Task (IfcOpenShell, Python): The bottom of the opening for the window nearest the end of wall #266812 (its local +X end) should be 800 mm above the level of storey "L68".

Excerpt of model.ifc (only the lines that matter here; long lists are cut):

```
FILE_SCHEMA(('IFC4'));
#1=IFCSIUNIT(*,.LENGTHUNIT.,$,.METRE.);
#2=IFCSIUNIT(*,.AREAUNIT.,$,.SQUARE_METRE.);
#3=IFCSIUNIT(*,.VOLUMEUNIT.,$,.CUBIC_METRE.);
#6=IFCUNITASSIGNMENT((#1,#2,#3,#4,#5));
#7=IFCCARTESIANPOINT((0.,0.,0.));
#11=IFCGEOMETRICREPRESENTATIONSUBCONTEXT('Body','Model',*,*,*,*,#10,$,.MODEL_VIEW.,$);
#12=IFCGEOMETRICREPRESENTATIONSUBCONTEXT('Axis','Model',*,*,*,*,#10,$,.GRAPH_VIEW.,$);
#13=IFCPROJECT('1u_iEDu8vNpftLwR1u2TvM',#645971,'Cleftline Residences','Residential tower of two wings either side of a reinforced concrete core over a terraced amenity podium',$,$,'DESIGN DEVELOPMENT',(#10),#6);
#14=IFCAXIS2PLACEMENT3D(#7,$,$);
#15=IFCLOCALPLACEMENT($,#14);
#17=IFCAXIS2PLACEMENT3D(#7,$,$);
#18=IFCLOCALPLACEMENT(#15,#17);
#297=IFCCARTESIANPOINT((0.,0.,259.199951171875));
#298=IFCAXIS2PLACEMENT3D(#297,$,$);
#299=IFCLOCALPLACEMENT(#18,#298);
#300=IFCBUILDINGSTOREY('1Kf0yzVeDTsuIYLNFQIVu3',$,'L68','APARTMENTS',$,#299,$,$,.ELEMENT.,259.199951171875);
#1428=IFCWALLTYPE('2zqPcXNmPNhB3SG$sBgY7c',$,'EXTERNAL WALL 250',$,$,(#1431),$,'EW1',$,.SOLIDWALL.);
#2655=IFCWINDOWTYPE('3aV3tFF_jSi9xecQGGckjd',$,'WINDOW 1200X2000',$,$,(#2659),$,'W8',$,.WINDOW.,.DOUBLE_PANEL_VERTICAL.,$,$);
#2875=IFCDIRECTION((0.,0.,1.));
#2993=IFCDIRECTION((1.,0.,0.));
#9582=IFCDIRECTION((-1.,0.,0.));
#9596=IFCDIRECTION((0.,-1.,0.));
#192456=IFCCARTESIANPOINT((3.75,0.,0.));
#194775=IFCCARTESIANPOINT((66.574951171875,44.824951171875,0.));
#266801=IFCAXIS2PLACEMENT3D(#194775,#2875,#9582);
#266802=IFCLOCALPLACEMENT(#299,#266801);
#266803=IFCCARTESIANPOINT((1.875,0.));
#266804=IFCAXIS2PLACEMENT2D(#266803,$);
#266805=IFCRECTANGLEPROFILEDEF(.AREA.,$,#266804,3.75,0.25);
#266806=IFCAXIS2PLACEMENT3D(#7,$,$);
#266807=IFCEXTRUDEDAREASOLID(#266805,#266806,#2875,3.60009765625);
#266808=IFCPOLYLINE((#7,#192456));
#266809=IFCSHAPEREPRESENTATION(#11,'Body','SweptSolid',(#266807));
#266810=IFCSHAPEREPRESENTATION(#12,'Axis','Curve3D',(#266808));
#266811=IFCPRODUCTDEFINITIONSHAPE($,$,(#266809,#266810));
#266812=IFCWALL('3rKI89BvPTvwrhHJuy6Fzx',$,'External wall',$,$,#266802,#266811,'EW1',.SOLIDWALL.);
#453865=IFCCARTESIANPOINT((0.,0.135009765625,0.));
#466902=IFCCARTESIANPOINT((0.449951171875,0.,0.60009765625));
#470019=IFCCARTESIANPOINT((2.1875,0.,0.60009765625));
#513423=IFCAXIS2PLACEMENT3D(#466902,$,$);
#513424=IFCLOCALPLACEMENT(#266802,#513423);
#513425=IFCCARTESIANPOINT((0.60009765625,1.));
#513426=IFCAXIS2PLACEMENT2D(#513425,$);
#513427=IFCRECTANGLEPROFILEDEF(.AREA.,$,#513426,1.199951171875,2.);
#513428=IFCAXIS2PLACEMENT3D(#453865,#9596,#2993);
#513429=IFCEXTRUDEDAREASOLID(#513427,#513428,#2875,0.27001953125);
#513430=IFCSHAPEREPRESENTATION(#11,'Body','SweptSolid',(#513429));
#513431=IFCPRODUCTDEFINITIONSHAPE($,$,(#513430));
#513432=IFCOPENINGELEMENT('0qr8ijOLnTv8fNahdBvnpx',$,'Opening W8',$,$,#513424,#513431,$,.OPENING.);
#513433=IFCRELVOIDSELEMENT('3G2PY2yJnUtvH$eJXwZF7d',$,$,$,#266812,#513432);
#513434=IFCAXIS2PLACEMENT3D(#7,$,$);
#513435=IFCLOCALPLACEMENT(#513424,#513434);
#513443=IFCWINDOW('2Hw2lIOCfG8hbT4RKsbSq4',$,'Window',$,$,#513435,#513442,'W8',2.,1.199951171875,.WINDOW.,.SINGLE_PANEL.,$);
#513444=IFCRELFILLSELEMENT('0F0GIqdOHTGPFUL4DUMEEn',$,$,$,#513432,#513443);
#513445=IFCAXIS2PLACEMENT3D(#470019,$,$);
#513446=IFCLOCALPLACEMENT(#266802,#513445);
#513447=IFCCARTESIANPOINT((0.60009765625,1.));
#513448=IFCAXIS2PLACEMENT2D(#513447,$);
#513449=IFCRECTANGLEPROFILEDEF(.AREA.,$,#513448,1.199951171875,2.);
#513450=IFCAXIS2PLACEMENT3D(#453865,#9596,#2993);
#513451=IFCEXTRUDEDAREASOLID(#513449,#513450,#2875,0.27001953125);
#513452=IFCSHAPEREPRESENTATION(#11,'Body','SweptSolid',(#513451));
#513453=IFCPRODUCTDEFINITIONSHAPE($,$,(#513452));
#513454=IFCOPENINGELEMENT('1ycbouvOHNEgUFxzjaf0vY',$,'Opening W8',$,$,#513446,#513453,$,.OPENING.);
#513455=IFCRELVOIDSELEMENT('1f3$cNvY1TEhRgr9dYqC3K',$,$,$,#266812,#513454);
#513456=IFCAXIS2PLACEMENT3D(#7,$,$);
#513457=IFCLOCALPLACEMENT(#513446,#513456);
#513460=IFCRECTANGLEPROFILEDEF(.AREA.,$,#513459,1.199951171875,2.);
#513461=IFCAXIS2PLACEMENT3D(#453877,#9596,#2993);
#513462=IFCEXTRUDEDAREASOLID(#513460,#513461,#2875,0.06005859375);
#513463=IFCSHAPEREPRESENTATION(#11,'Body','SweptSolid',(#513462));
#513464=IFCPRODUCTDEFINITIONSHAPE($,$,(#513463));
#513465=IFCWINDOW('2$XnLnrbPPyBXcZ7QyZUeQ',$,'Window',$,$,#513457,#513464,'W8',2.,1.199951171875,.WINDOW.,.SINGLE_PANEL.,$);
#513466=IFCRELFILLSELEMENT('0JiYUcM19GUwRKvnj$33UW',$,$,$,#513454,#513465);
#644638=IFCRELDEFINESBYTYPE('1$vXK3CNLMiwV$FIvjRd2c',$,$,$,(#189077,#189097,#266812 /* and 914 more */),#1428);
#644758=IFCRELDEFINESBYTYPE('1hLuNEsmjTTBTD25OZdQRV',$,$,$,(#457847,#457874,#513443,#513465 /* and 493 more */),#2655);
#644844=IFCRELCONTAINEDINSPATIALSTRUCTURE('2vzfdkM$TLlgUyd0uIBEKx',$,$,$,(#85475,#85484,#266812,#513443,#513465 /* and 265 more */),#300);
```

```python
import numpy as np
import ifcopenshell
import ifcopenshell.api.geometry
import ifcopenshell.geom
import ifcopenshell.util.element
import ifcopenshell.util.placement
import ifcopenshell.util.shape
import ifcopenshell.util.unit

model = ifcopenshell.open("model.ifc")
unit_scale = ifcopenshell.util.unit.calculate_unit_scale(model)

window = model.by_guid("2$XnLnrbPPyBXcZ7QyZUeQ")
opening = window.FillsVoids[0].RelatingOpeningElement
storey = ifcopenshell.util.element.get_container(window, ifc_class="IfcBuildingStorey")
level = ifcopenshell.util.placement.get_local_placement(storey.ObjectPlacement)[2, 3]

# The opening's origin need not be at the sill, so measure its lowest point.
shape = ifcopenshell.geom.create_shape(ifcopenshell.geom.settings(), opening)
bottom = ifcopenshell.util.shape.get_shape_bottom_elevation(shape, shape.geometry) / unit_scale
dz = level + 0.8 / unit_scale - bottom

shift = np.array([0.0, 0.0, dz])
# The window is placed relative to its opening, so it follows when the opening moves.
matrix = ifcopenshell.util.placement.get_local_placement(opening.ObjectPlacement)
matrix[:3, 3] += shift
ifcopenshell.api.geometry.edit_object_placement(
    model, product=opening, matrix=matrix, is_si=False, should_transform_children=True
)

print(f"moved by {dz * unit_scale:+.3f} m")

model.write("model_rev.ifc")
```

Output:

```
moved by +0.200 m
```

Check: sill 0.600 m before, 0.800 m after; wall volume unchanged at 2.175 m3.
